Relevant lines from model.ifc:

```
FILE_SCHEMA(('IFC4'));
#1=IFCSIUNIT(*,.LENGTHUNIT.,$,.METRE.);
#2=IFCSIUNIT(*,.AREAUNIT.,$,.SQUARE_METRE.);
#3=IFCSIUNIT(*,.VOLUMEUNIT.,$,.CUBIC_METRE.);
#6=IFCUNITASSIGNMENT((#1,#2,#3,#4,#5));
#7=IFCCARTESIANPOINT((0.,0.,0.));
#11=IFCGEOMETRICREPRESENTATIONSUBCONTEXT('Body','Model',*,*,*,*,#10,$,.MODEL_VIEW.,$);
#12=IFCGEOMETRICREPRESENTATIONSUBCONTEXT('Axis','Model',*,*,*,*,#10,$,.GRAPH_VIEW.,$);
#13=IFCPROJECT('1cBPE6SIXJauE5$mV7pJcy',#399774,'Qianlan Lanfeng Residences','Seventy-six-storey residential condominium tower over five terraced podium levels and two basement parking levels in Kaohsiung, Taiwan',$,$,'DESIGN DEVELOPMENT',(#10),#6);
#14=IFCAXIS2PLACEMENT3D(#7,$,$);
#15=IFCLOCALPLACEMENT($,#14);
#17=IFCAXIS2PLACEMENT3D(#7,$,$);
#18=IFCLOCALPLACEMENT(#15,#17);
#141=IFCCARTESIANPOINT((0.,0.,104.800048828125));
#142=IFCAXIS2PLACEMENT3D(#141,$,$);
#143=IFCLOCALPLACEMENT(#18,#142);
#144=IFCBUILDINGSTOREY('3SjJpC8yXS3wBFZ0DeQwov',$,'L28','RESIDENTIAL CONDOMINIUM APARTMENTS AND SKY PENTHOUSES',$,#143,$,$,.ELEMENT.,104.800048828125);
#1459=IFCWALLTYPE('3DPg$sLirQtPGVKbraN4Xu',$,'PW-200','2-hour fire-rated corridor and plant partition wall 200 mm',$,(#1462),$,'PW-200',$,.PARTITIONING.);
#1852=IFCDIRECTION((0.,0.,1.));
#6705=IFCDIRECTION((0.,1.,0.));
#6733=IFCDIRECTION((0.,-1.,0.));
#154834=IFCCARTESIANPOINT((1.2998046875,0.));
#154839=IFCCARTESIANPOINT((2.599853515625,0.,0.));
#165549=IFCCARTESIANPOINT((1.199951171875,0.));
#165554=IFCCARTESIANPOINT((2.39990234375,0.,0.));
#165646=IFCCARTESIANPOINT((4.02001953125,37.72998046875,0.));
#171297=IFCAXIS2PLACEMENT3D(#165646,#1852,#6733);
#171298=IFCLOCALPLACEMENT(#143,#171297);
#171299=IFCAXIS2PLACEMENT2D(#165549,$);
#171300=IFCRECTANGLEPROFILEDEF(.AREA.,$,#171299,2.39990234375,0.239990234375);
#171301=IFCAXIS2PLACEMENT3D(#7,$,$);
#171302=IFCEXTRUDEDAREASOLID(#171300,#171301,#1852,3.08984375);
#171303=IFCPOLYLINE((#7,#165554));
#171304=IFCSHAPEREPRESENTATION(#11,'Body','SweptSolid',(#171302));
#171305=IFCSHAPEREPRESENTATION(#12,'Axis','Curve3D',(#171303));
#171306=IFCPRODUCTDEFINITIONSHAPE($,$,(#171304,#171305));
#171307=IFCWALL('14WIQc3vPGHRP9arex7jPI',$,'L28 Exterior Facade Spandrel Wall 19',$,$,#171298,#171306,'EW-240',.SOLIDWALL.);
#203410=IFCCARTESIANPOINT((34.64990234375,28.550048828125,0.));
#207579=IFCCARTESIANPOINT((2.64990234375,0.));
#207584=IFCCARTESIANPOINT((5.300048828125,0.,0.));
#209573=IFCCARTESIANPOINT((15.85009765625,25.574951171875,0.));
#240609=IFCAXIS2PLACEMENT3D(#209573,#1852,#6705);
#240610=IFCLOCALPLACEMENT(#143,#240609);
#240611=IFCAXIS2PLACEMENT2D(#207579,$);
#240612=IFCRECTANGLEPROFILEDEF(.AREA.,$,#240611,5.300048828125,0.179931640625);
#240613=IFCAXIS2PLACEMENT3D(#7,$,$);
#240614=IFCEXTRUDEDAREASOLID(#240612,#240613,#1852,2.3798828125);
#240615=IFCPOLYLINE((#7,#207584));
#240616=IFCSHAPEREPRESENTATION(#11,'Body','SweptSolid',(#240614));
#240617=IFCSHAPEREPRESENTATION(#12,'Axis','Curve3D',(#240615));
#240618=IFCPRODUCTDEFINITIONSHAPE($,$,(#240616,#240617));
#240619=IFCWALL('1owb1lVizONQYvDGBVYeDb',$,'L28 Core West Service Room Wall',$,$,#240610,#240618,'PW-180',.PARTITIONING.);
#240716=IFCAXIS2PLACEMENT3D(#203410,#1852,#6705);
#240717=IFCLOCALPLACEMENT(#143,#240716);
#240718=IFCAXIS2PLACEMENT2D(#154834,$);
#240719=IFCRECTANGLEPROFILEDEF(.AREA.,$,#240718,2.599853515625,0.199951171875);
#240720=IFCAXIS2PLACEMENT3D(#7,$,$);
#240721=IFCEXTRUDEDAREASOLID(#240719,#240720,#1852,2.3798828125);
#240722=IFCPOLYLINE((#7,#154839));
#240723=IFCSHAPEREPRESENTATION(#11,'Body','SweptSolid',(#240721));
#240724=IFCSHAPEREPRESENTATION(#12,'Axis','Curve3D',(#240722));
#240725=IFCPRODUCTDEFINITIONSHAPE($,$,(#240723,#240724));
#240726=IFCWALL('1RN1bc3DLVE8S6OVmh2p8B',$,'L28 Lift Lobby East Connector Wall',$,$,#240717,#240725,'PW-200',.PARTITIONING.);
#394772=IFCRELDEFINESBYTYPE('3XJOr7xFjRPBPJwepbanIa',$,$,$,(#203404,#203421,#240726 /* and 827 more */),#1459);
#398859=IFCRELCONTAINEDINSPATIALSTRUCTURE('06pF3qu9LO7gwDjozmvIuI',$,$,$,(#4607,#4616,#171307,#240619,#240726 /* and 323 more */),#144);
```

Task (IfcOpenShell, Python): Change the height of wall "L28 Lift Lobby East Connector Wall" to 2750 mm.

```python
import ifcopenshell
import ifcopenshell.geom
import ifcopenshell.util.representation
import ifcopenshell.util.shape
import ifcopenshell.util.unit

model = ifcopenshell.open("model.ifc")
unit_scale = ifcopenshell.util.unit.calculate_unit_scale(model)
settings = ifcopenshell.geom.settings()


def volume(element):
    """Net volume in cubic metres, openings subtracted."""
    shape = ifcopenshell.geom.create_shape(settings, element)
    return ifcopenshell.util.shape.get_volume(shape.geometry)


wall = model.by_guid("1RN1bc3DLVE8S6OVmh2p8B")
before = volume(wall)

body = ifcopenshell.util.representation.get_representation(wall, "Model", "Body")
solid = body.Items[0]
old_height = solid.Depth
solid.Depth = 2.75 / unit_scale
after = volume(wall)

print(f"height {old_height:g} -> {solid.Depth:g}, volume {before:.3f} -> {after:.3f} m3")

model.write("model-out.ifc")
```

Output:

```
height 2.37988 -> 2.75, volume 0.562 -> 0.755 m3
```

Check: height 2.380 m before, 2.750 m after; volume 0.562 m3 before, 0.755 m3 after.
